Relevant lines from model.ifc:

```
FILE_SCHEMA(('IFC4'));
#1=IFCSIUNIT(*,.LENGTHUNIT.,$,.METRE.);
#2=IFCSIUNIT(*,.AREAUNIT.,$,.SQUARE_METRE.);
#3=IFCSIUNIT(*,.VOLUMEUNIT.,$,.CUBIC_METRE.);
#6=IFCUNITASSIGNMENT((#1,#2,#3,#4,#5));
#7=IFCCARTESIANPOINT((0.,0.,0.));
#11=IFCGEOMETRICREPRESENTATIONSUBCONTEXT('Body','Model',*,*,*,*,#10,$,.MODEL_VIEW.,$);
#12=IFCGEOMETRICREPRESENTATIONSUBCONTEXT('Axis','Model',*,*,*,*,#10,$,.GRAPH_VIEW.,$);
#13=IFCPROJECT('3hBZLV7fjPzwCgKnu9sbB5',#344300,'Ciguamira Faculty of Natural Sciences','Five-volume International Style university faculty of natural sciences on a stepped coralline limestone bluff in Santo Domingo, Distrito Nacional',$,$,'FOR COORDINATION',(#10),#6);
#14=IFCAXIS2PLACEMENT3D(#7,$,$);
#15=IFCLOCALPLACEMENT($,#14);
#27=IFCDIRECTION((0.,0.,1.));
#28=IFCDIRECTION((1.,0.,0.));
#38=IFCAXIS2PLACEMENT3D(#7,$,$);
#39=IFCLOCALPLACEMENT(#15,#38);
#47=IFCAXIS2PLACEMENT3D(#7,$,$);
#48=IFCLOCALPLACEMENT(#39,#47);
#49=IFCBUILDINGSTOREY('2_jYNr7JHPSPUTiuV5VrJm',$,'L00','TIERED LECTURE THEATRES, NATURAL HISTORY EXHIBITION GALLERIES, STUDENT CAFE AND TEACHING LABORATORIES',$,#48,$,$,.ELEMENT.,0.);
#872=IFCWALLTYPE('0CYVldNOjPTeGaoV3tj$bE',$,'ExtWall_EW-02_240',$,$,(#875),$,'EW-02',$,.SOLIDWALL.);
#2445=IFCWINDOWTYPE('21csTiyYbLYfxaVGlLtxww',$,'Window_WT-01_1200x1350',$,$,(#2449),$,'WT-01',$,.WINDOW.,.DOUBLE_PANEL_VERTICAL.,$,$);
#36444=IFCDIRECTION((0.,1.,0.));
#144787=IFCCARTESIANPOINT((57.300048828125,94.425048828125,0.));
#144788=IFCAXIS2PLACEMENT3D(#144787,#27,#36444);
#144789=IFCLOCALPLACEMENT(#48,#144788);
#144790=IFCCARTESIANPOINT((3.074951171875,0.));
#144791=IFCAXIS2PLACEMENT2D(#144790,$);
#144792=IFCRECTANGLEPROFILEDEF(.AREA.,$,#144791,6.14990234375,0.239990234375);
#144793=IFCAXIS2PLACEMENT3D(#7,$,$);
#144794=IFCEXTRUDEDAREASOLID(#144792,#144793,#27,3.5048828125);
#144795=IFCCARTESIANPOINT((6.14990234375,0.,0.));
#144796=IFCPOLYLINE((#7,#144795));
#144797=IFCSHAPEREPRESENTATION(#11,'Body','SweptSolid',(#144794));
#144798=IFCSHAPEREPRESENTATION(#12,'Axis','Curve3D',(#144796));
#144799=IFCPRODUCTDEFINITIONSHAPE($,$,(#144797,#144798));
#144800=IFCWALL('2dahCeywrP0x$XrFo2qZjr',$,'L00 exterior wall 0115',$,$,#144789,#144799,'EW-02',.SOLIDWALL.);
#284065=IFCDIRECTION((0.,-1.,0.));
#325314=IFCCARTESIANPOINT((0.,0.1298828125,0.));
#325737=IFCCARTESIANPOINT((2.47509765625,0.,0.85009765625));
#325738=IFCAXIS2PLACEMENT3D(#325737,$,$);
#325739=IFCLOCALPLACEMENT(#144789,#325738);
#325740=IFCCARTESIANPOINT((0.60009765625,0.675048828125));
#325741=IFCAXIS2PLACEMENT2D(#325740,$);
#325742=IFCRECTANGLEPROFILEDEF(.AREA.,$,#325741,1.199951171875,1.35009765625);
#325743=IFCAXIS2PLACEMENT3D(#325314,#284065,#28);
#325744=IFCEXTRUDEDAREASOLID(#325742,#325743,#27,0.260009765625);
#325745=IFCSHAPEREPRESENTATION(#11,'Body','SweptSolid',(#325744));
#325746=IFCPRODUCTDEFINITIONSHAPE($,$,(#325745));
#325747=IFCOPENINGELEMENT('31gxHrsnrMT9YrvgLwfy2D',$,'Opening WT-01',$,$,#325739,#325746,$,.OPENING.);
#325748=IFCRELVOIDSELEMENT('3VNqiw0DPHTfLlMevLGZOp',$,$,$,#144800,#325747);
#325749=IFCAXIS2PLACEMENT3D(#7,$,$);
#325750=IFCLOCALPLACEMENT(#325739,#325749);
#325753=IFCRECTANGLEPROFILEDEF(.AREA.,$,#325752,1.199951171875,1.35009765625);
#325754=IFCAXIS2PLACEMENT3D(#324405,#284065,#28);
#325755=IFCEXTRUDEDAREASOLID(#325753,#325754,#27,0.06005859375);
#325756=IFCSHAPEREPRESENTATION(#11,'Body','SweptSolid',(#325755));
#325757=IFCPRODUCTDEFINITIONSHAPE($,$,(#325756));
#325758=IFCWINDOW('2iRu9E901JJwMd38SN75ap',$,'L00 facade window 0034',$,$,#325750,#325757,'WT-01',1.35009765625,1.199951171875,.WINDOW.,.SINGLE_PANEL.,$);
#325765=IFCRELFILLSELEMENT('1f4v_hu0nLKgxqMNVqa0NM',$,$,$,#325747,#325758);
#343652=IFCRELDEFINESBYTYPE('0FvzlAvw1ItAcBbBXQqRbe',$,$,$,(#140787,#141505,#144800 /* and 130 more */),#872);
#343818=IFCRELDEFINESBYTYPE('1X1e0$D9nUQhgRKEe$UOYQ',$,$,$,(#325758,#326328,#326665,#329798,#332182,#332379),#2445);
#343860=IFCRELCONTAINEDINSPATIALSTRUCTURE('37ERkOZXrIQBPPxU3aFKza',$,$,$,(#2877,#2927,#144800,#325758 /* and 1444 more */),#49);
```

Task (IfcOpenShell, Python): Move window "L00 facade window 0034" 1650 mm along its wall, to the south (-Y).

```python
import ifcopenshell
import ifcopenshell.api.geometry
import ifcopenshell.util.placement
import ifcopenshell.util.unit

model = ifcopenshell.open("model.ifc")
unit_scale = ifcopenshell.util.unit.calculate_unit_scale(model)

window = model.by_guid("2iRu9E901JJwMd38SN75ap")
opening = window.FillsVoids[0].RelatingOpeningElement
wall = opening.VoidsElements[0].RelatingBuildingElement

wall_matrix = ifcopenshell.util.placement.get_local_placement(wall.ObjectPlacement)
shift = wall_matrix[:3, 0] * -1.65 / unit_scale
before = ifcopenshell.util.placement.get_local_placement(window.ObjectPlacement)[:3, 3].copy()

# The window is placed relative to its opening, so it follows when the opening moves.
matrix = ifcopenshell.util.placement.get_local_placement(opening.ObjectPlacement)
matrix[:3, 3] += shift
ifcopenshell.api.geometry.edit_object_placement(
    model, product=opening, matrix=matrix, is_si=False, should_transform_children=True
)

after = ifcopenshell.util.placement.get_local_placement(window.ObjectPlacement)[:3, 3]
print("window moved by", (after - before).round(3) + 0.0)

model.write("model_edited.ifc")
```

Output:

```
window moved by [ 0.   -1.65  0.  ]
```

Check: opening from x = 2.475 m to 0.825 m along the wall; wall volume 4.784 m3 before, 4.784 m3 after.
